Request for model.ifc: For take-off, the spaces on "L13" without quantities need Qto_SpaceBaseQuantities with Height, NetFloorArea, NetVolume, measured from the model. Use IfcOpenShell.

First a look at what the model holds.

```python
import ifcopenshell
import ifcopenshell.util.element
import ifcopenshell.util.unit

model = ifcopenshell.open("model.ifc")
print(model.schema)
for unit_type in ("LENGTHUNIT", "AREAUNIT", "VOLUMEUNIT"):
    print(unit_type, ifcopenshell.util.unit.calculate_unit_scale(model, unit_type))
storey = next(s for s in model.by_type("IfcBuildingStorey") if s.Name == "L13")
spaces = [e for e in ifcopenshell.util.element.get_decomposition(storey) if e.is_a("IfcSpace")]
for e in sorted(spaces, key=lambda e: e.id()):
    print(e.id(), e.is_a(), e.Name, list(ifcopenshell.util.element.get_psets(e, qtos_only=True)), sep=" | ")
```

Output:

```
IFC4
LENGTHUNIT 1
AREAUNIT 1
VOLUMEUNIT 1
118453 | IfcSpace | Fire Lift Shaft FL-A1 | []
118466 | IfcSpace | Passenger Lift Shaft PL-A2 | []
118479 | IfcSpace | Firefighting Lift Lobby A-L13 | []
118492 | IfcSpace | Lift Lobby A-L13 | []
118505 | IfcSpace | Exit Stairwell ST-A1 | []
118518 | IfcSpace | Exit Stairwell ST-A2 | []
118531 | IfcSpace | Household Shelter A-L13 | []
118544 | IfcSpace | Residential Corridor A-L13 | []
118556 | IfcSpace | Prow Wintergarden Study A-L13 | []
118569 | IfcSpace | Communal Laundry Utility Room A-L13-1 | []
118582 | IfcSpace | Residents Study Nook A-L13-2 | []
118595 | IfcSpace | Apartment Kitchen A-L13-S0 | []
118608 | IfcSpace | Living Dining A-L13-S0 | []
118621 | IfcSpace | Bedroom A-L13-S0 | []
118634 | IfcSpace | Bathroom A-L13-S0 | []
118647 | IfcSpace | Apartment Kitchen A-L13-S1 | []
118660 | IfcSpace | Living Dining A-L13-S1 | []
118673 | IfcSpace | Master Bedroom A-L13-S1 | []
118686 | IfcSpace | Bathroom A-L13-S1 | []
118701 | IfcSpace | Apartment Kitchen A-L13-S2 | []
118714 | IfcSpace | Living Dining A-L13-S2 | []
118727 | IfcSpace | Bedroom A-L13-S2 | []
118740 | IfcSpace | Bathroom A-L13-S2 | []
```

```python
import ifcopenshell
import ifcopenshell.api.pset
import ifcopenshell.geom
import ifcopenshell.util.element
import ifcopenshell.util.shape
import ifcopenshell.util.unit

model = ifcopenshell.open("model.ifc")
unit_scale = ifcopenshell.util.unit.calculate_unit_scale(model)
area_scale = ifcopenshell.util.unit.calculate_unit_scale(model, "AREAUNIT")
volume_scale = ifcopenshell.util.unit.calculate_unit_scale(model, "VOLUMEUNIT")
settings = ifcopenshell.geom.settings()

storey = next(s for s in model.by_type("IfcBuildingStorey") if s.Name == "L13")
spaces = [e for e in ifcopenshell.util.element.get_decomposition(storey) if e.is_a("IfcSpace")]

for e in sorted(spaces, key=lambda e: e.id()):
    if ifcopenshell.util.element.get_psets(e, qtos_only=True, should_inherit=False):
        continue
    # Geometry comes back in metres, in the element's own axes.
    shape = ifcopenshell.geom.create_shape(settings, e)
    values = {
        "Height": ifcopenshell.util.shape.get_z(shape.geometry) / unit_scale,
        "NetFloorArea": ifcopenshell.util.shape.get_footprint_area(shape.geometry) / area_scale,
        "NetVolume": ifcopenshell.util.shape.get_volume(shape.geometry) / volume_scale,
    }
    qto = ifcopenshell.api.pset.add_qto(model, product=e, name="Qto_SpaceBaseQuantities")
    ifcopenshell.api.pset.edit_qto(model, qto=qto, properties=values)
    print(e.id(), {k: round(v, 3) for k, v in values.items()})

model.write("model_v2.ifc")
```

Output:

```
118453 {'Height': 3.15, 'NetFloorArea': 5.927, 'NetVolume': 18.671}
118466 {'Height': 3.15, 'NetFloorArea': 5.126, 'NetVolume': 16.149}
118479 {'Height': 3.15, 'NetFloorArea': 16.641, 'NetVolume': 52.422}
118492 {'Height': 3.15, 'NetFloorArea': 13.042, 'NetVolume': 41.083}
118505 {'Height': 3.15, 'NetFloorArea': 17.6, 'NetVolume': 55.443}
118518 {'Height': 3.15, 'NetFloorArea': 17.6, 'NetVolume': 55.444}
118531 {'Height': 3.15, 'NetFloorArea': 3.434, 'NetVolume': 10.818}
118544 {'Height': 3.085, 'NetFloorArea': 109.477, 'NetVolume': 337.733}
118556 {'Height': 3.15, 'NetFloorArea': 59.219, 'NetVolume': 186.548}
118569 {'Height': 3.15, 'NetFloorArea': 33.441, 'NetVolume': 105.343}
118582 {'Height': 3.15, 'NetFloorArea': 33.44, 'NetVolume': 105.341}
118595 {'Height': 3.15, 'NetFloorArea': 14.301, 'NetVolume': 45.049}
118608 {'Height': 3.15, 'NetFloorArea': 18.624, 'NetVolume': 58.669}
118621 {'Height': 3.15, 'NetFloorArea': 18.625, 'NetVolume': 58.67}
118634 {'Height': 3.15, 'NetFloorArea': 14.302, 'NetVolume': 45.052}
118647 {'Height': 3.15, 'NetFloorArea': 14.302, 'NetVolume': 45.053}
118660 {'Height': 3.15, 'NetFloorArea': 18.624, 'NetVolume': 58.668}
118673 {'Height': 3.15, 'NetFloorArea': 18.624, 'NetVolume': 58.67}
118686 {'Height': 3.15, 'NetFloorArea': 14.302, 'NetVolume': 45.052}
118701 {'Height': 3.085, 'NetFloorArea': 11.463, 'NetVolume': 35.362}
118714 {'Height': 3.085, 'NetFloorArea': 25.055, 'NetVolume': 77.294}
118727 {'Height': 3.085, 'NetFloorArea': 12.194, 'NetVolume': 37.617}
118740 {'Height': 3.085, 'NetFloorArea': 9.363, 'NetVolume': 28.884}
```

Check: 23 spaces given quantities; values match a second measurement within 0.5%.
